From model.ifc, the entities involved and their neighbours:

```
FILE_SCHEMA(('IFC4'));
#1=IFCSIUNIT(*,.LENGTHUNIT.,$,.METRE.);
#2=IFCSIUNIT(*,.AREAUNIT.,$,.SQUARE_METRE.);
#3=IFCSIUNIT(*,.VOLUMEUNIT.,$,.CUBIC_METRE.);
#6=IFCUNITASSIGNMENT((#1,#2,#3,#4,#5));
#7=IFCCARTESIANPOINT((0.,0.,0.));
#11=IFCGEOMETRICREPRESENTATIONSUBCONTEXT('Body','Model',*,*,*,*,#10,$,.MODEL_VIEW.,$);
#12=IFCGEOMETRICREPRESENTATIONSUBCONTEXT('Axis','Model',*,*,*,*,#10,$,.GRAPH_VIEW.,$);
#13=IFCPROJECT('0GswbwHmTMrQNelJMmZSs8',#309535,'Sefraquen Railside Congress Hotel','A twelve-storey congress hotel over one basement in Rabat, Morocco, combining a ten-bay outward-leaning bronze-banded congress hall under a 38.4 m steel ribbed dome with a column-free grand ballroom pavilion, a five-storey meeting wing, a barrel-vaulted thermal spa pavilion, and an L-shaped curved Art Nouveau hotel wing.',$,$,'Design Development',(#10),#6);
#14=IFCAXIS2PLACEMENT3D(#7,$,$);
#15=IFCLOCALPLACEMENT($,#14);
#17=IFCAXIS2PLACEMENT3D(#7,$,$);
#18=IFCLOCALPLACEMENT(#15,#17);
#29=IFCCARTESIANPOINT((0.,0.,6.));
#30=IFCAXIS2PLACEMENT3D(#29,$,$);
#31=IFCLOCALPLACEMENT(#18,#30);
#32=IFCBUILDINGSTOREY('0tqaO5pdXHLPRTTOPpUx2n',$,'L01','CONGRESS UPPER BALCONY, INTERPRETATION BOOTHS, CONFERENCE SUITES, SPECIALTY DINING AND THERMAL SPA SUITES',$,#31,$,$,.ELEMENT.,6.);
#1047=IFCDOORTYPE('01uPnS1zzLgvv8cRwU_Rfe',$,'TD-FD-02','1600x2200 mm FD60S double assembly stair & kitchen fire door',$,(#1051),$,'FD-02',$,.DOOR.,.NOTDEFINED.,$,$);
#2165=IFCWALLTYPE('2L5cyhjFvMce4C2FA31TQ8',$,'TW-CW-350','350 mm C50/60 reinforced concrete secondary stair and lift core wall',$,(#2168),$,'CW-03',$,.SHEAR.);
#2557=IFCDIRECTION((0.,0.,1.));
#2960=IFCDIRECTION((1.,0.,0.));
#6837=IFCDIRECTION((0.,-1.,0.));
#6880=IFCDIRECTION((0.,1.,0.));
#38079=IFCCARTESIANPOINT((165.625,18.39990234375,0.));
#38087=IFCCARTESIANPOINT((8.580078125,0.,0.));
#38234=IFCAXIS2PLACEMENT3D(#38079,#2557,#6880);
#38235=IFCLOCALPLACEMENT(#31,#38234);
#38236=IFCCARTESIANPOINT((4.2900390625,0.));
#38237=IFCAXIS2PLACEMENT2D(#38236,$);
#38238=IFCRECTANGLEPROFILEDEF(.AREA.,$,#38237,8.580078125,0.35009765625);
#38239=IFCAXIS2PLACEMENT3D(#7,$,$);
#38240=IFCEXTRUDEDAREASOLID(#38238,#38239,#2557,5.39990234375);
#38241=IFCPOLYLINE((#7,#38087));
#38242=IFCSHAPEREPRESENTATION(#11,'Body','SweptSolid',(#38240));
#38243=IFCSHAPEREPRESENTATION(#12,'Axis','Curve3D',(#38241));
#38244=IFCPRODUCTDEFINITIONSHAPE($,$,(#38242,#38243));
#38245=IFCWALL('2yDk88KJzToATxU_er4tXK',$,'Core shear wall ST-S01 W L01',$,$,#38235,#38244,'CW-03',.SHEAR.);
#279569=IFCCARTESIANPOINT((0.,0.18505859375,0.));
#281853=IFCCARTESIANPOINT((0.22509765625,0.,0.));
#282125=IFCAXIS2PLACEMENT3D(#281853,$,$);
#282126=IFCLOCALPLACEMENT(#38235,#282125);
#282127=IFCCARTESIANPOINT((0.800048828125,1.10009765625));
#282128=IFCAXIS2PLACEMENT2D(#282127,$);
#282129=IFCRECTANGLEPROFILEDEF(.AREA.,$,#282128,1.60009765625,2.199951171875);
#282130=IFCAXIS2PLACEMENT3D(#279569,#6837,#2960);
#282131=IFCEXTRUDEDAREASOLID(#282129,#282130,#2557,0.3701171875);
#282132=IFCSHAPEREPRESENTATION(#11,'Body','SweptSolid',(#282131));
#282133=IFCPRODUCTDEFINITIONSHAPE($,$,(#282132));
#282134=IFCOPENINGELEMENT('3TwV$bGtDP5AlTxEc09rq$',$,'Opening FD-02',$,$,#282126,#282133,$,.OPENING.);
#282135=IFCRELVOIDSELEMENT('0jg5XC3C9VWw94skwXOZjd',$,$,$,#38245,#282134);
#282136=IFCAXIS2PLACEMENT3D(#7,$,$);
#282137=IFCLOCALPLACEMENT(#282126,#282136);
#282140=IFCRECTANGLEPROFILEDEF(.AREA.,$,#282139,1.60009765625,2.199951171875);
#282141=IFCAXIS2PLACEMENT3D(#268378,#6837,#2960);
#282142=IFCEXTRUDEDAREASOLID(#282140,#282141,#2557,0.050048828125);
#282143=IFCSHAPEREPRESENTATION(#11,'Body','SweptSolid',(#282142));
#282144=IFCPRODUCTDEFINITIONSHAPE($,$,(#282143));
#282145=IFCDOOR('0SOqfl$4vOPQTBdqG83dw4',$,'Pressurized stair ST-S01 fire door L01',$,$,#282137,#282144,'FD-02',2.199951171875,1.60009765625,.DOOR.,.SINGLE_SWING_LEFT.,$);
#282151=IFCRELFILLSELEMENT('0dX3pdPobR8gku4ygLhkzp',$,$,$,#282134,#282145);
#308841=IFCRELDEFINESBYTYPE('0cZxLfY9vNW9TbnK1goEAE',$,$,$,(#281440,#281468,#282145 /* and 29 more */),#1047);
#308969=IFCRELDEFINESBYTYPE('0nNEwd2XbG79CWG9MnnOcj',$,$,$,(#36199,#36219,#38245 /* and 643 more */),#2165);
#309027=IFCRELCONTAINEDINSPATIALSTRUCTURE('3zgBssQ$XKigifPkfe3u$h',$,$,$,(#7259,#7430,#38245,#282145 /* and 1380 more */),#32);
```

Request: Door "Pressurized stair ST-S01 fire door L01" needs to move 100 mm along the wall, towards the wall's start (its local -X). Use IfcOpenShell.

```python
import ifcopenshell
import ifcopenshell.api.geometry
import ifcopenshell.util.placement
import ifcopenshell.util.unit

model = ifcopenshell.open("model.ifc")
unit_scale = ifcopenshell.util.unit.calculate_unit_scale(model)

door = model.by_id(282145)
opening = door.FillsVoids[0].RelatingOpeningElement
wall = opening.VoidsElements[0].RelatingBuildingElement

wall_matrix = ifcopenshell.util.placement.get_local_placement(wall.ObjectPlacement)
shift = wall_matrix[:3, 0] * -0.1 / unit_scale
before = ifcopenshell.util.placement.get_local_placement(door.ObjectPlacement)[:3, 3].copy()

# The door is placed relative to its opening, so it follows when the opening moves.
matrix = ifcopenshell.util.placement.get_local_placement(opening.ObjectPlacement)
matrix[:3, 3] += shift
ifcopenshell.api.geometry.edit_object_placement(
    model, product=opening, matrix=matrix, is_si=False, should_transform_children=True
)

after = ifcopenshell.util.placement.get_local_placement(door.ObjectPlacement)[:3, 3]
print("door moved by", (after - before).round(3) + 0.0)

model.write("model-out.ifc")
```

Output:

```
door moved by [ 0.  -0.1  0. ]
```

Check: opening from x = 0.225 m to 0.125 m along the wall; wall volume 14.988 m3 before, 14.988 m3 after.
